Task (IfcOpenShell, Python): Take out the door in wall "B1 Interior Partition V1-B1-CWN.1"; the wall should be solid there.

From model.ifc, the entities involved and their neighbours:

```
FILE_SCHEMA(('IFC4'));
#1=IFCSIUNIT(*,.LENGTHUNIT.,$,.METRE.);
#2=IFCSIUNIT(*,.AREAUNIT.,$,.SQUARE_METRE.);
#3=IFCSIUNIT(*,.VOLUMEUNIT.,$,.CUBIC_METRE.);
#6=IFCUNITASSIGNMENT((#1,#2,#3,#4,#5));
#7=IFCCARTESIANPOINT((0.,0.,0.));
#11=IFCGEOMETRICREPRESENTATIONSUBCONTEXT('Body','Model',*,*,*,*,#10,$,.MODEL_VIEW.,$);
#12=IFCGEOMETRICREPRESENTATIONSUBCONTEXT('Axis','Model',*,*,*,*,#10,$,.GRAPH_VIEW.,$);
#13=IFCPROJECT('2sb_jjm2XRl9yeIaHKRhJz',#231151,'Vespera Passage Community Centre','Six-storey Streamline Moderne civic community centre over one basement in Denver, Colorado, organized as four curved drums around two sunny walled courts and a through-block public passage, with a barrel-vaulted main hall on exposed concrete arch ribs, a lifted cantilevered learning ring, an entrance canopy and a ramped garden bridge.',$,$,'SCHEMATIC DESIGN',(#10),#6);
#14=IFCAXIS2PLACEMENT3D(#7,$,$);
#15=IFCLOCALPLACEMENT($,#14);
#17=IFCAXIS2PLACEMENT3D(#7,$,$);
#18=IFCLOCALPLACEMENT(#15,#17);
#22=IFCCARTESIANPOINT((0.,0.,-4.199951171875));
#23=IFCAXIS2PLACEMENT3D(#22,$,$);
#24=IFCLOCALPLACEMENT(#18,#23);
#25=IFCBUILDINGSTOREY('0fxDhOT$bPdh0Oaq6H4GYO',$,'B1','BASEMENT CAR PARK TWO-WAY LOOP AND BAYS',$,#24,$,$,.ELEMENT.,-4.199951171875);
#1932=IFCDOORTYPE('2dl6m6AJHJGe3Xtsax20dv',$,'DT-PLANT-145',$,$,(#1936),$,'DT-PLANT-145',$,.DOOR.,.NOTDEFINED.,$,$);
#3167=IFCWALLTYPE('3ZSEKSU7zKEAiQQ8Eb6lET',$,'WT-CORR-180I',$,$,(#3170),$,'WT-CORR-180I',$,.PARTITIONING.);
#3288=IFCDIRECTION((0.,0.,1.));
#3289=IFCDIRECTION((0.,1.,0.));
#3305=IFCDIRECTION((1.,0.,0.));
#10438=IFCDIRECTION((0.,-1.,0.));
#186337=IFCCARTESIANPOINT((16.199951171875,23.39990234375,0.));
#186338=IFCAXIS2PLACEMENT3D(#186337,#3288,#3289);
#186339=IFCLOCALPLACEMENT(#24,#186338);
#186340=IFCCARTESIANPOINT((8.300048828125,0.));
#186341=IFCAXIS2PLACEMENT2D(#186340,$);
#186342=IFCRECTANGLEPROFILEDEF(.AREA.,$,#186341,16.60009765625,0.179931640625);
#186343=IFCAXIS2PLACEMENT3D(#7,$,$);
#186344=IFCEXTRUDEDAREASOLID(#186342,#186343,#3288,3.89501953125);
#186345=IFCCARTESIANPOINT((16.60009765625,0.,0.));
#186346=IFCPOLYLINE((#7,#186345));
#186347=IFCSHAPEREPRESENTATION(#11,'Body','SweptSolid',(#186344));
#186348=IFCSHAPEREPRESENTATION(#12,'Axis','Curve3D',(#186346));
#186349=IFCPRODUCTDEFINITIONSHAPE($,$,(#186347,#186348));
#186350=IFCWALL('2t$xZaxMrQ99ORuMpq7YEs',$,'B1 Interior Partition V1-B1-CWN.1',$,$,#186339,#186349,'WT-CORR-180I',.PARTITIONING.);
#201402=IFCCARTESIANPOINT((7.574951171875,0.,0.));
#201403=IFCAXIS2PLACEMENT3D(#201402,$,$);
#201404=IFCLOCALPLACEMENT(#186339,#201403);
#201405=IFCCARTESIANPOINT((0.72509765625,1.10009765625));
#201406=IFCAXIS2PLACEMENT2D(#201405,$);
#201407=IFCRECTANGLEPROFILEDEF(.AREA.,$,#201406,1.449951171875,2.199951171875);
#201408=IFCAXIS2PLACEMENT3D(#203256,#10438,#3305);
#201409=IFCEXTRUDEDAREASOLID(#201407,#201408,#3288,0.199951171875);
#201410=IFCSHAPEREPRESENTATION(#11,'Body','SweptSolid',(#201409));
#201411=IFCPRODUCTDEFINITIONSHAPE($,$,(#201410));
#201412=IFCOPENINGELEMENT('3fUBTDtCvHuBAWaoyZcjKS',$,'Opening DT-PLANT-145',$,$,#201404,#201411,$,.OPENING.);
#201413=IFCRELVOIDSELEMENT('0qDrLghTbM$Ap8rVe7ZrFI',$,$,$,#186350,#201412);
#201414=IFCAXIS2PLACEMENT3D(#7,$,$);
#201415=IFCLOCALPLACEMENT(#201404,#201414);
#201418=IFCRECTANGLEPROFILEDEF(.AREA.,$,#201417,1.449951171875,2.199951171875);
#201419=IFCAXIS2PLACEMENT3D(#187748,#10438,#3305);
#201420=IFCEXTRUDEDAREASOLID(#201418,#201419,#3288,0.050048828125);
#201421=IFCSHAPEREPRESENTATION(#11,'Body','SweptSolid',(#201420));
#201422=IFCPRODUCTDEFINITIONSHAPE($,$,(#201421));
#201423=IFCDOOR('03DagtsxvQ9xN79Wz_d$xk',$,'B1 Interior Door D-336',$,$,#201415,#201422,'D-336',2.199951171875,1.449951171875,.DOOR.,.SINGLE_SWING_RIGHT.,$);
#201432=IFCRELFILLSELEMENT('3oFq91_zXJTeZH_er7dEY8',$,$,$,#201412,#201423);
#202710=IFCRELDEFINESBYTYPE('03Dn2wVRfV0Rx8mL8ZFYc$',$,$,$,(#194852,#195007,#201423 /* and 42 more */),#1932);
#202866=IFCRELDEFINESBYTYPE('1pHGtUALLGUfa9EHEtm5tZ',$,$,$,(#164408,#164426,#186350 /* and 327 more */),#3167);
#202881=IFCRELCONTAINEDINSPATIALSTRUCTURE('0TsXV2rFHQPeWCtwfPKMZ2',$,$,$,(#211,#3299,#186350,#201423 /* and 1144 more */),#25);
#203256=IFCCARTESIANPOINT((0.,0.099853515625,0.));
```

```python
import ifcopenshell
import ifcopenshell.api.feature
import ifcopenshell.api.root
import ifcopenshell.geom
import ifcopenshell.util.shape

model = ifcopenshell.open("model.ifc")
settings = ifcopenshell.geom.settings()


def volume(element):
    """Net volume in cubic metres, openings subtracted."""
    shape = ifcopenshell.geom.create_shape(settings, element)
    return ifcopenshell.util.shape.get_volume(shape.geometry)


door = model.by_guid("03DagtsxvQ9xN79Wz_d$xk")
opening = door.FillsVoids[0].RelatingOpeningElement
wall = opening.VoidsElements[0].RelatingBuildingElement
before = volume(wall)

ifcopenshell.api.root.remove_product(model, product=door)
ifcopenshell.api.feature.remove_feature(model, feature=opening)

after = volume(wall)

print(f"wall volume {before:.3f} -> {after:.3f} m3")

model.write("model_edited.ifc")
```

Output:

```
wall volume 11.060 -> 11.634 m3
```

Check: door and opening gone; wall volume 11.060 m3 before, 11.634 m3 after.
